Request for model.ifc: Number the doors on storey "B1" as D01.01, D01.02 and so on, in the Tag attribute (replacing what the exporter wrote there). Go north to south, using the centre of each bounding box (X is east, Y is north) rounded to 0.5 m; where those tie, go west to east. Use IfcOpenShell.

First a look at what the model holds.

```python
import ifcopenshell
import ifcopenshell.util.element
import ifcopenshell.util.placement

model = ifcopenshell.open("model.ifc")
print(model.schema)
storey = next(s for s in model.by_type("IfcBuildingStorey") if s.Name == "B1")
doors = [e for e in ifcopenshell.util.element.get_decomposition(storey) if e.is_a("IfcDoor")]
for e in sorted(doors, key=lambda e: e.id()):
    origin = ifcopenshell.util.placement.get_local_placement(e.ObjectPlacement)[:3, 3]
    print(e.id(), e.Tag, e.Name, origin.round(2) + 0.0, sep=" | ")
```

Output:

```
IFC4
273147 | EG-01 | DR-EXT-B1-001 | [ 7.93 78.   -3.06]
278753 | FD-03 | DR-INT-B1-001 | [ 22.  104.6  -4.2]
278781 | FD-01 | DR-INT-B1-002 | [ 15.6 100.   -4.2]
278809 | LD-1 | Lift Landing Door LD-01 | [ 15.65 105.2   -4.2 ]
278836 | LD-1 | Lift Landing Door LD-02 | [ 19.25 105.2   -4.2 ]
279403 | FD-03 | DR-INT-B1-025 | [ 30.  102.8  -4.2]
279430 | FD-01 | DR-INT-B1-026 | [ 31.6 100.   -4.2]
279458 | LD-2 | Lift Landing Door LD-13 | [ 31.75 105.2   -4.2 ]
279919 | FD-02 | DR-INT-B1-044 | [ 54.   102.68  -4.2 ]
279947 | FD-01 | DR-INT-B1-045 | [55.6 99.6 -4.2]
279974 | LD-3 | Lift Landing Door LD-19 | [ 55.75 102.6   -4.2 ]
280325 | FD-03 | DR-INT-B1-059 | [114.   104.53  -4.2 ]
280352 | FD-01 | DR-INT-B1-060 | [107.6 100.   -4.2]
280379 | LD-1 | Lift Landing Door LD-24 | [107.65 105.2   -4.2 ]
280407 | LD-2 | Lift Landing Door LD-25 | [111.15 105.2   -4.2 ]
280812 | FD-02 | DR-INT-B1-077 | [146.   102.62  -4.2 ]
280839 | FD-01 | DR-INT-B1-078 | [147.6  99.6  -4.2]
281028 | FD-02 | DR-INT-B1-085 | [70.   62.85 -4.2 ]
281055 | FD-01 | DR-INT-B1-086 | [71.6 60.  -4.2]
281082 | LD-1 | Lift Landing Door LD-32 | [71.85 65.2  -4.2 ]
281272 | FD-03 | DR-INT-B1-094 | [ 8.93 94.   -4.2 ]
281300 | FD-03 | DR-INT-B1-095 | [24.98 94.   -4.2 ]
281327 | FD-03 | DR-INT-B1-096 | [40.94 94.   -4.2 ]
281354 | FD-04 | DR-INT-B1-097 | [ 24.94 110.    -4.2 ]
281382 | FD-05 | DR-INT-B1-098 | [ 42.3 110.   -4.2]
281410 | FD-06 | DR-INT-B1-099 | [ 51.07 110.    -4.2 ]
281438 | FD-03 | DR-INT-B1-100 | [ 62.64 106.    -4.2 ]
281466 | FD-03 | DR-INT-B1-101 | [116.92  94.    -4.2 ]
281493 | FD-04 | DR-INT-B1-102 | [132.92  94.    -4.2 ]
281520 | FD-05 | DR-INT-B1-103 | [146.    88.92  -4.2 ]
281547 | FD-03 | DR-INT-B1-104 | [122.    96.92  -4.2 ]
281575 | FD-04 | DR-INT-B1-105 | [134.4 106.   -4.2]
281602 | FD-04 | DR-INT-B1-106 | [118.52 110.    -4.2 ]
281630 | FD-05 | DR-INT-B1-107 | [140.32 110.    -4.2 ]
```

```python
import ifcopenshell
import ifcopenshell.geom
import ifcopenshell.util.element
import ifcopenshell.util.shape

model = ifcopenshell.open("model.ifc")
settings = ifcopenshell.geom.settings()
settings.set("use-world-coords", True)


def centre(element):
    shape = ifcopenshell.geom.create_shape(settings, element)
    return ifcopenshell.util.shape.get_bbox_centroid(shape.geometry)


storey = next(s for s in model.by_type("IfcBuildingStorey") if s.Name == "B1")
doors = [e for e in ifcopenshell.util.element.get_decomposition(storey) if e.is_a("IfcDoor")]

# Insertion points can sit at a corner or the storey origin, so sort by the geometry (in metres).
centres = {e: centre(e) for e in doors}
doors.sort(key=lambda e: (-round(centres[e][1] / 0.5), centres[e][0]))

for i, e in enumerate(doors, start=1):
    number = f"D01.{i:02d}"
    e.Tag = number
    print(e.id(), number)

model.write("model_rev.ifc")
```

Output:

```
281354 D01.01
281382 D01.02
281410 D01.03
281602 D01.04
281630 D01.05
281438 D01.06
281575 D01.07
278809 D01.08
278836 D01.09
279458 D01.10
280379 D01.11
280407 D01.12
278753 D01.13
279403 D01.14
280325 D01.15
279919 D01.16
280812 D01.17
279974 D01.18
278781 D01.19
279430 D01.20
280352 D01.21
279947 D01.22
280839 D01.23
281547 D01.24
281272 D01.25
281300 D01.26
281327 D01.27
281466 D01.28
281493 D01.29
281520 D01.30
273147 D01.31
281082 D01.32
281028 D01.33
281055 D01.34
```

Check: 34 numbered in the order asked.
